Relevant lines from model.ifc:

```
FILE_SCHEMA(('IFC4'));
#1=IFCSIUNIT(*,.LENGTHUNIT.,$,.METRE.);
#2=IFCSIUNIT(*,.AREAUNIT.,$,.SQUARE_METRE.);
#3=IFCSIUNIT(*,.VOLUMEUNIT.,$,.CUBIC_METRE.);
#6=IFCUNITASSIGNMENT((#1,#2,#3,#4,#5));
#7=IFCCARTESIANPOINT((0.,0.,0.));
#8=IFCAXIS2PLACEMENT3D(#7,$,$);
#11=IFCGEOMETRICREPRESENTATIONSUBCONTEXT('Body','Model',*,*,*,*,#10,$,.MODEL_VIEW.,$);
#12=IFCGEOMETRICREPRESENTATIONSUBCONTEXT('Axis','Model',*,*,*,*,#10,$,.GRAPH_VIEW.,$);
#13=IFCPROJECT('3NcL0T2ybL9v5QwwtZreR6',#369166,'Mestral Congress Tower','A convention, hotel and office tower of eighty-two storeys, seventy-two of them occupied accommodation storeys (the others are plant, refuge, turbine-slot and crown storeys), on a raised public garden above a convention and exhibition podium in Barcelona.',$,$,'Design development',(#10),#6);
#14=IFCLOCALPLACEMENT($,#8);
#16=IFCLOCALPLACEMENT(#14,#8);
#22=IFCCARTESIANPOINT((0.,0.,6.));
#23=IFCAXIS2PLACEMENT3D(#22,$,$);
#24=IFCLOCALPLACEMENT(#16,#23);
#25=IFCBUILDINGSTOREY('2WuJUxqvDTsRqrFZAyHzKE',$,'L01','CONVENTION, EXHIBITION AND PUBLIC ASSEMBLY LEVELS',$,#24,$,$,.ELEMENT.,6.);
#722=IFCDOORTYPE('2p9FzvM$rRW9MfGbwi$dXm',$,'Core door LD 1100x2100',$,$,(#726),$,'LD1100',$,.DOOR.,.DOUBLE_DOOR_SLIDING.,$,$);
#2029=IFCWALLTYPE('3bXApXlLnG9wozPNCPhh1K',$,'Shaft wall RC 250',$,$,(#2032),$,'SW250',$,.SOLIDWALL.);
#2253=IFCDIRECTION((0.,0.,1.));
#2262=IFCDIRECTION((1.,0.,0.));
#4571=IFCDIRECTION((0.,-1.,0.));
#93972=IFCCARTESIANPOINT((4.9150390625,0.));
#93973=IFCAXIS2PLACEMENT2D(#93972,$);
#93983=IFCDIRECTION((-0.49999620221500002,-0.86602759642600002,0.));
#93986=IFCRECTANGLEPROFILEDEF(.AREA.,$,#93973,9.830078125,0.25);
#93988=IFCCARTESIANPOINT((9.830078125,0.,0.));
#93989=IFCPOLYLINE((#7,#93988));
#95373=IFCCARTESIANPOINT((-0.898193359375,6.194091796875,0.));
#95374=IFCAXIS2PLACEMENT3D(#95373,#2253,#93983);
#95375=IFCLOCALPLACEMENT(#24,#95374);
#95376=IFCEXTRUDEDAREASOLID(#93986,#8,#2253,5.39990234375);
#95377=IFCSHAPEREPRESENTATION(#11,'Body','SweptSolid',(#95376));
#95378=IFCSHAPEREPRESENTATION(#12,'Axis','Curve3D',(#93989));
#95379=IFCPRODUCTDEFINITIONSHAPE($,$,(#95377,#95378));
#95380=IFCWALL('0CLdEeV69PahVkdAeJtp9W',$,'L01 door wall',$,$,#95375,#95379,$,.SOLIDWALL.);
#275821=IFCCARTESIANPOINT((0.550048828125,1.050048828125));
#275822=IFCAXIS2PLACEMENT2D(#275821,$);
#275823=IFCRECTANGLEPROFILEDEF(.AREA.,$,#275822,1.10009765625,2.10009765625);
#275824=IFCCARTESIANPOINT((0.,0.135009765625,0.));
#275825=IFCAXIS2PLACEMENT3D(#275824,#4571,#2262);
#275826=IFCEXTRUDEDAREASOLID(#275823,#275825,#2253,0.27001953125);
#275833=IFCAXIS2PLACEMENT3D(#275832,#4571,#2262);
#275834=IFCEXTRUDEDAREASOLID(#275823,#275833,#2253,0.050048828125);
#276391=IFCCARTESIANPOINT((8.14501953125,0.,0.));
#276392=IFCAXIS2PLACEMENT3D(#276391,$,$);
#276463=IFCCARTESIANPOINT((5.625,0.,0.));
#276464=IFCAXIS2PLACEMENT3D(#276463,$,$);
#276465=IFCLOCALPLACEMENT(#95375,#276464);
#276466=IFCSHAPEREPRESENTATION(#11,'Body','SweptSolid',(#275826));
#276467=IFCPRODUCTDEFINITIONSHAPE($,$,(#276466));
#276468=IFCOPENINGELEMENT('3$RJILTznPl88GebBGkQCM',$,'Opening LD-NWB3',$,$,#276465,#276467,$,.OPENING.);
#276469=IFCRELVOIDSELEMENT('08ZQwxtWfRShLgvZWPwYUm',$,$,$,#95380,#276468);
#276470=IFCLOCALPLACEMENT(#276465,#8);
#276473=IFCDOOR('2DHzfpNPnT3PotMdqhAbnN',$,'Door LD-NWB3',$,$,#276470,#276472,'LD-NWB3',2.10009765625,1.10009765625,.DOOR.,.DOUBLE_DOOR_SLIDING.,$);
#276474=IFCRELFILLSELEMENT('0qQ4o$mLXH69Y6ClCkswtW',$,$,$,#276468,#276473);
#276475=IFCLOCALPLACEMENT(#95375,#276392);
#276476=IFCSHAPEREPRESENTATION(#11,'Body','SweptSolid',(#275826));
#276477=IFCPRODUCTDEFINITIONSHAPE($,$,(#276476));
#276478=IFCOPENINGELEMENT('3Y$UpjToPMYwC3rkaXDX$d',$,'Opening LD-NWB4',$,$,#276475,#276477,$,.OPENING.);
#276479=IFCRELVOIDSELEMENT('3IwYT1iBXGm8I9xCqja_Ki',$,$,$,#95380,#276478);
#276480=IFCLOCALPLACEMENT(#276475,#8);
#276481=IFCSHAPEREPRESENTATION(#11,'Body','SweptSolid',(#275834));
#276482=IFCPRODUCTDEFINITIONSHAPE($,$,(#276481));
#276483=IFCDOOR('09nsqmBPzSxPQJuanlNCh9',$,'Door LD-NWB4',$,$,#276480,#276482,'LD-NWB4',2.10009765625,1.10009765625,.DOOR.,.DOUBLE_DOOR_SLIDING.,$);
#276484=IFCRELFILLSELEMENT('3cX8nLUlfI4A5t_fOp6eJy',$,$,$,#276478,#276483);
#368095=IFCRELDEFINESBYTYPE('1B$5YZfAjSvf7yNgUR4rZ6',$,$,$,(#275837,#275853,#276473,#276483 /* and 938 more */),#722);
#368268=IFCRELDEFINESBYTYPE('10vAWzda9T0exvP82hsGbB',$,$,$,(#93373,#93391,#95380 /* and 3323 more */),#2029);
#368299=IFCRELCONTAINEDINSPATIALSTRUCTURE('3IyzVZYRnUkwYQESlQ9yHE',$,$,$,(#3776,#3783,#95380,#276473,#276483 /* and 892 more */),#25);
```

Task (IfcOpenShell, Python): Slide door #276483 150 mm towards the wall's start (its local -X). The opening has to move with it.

```python
import ifcopenshell
import ifcopenshell.api.geometry
import ifcopenshell.util.placement
import ifcopenshell.util.unit

model = ifcopenshell.open("model.ifc")
unit_scale = ifcopenshell.util.unit.calculate_unit_scale(model)

door = model.by_guid("09nsqmBPzSxPQJuanlNCh9")
opening = door.FillsVoids[0].RelatingOpeningElement
wall = opening.VoidsElements[0].RelatingBuildingElement

wall_matrix = ifcopenshell.util.placement.get_local_placement(wall.ObjectPlacement)
shift = wall_matrix[:3, 0] * -0.15 / unit_scale
before = ifcopenshell.util.placement.get_local_placement(door.ObjectPlacement)[:3, 3].copy()

# The door is placed relative to its opening, so it follows when the opening moves.
matrix = ifcopenshell.util.placement.get_local_placement(opening.ObjectPlacement)
matrix[:3, 3] += shift
ifcopenshell.api.geometry.edit_object_placement(
    model, product=opening, matrix=matrix, is_si=False, should_transform_children=True
)

after = ifcopenshell.util.placement.get_local_placement(door.ObjectPlacement)[:3, 3]
print("door moved by", (after - before).round(3) + 0.0)

model.write("model-out.ifc")
```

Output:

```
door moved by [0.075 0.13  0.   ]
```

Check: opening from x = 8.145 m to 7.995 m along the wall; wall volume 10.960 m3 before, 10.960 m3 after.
